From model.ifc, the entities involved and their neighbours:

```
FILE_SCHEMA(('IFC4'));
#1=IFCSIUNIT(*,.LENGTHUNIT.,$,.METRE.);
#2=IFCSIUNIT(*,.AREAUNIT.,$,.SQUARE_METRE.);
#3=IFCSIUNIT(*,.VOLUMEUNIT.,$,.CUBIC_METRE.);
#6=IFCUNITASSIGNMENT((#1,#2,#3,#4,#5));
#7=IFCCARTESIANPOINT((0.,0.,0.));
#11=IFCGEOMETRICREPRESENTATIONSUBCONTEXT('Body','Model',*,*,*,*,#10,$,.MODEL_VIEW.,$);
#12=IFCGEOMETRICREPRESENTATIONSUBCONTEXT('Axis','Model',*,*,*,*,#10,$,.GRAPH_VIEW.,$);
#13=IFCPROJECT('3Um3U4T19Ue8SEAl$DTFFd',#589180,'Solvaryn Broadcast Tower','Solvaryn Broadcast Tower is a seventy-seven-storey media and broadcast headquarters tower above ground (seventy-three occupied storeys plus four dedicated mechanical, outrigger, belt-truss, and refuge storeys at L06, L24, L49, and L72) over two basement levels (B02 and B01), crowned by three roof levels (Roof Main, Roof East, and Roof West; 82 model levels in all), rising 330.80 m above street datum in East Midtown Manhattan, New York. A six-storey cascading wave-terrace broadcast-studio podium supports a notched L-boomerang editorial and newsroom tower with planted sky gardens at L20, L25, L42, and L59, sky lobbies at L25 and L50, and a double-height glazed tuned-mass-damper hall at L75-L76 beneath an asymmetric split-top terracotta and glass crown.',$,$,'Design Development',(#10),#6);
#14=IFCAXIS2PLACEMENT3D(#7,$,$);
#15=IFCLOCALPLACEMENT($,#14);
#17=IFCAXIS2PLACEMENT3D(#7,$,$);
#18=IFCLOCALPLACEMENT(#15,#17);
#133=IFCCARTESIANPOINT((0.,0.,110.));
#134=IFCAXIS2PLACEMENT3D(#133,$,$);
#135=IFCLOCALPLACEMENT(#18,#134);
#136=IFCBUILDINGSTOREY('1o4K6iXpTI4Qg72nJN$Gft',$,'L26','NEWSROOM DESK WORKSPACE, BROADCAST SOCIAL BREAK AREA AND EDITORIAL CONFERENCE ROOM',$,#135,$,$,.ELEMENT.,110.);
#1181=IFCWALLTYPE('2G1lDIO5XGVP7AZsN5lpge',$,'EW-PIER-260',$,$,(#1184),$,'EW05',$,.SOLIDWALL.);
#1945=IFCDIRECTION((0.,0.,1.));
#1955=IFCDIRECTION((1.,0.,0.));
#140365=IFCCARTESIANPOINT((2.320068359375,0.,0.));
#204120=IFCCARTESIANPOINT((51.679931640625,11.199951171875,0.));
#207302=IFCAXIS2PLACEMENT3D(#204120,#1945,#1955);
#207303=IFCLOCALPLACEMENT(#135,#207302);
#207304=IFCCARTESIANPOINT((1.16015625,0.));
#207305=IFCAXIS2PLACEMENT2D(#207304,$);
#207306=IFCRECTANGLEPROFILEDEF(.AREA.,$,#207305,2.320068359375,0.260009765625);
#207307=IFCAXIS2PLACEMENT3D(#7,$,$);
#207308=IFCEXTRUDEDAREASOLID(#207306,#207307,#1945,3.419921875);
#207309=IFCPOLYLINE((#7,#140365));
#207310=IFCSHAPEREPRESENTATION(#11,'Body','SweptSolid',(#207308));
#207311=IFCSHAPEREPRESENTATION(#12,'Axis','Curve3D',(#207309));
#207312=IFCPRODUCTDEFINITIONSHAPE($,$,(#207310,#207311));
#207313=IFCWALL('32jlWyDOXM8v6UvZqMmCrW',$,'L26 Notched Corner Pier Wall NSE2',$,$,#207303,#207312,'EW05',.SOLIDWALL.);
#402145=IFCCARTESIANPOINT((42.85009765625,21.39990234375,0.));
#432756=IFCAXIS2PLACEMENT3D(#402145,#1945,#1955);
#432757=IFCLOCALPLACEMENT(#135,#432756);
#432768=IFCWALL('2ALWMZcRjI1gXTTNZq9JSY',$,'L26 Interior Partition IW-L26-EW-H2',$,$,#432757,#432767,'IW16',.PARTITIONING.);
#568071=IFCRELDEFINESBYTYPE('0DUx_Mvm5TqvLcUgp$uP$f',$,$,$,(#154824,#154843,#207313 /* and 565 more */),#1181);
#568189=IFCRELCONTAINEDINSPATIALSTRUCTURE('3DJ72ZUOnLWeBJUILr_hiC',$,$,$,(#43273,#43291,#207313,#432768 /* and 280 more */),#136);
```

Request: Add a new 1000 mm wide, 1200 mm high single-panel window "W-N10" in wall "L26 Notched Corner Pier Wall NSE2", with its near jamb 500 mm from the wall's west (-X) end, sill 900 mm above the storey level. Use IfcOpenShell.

```python
import numpy as np
import ifcopenshell
import ifcopenshell.api.feature
import ifcopenshell.api.geometry
import ifcopenshell.api.root
import ifcopenshell.api.spatial
import ifcopenshell.geom
import ifcopenshell.util.element
import ifcopenshell.util.placement
import ifcopenshell.util.representation
import ifcopenshell.util.shape
import ifcopenshell.util.unit

model = ifcopenshell.open("model.ifc")
unit_scale = ifcopenshell.util.unit.calculate_unit_scale(model)
settings = ifcopenshell.geom.settings()


def volume(element):
    """Net volume in cubic metres, openings subtracted."""
    shape = ifcopenshell.geom.create_shape(settings, element)
    return ifcopenshell.util.shape.get_volume(shape.geometry)


wall = model.by_guid("32jlWyDOXM8v6UvZqMmCrW")
storey = ifcopenshell.util.element.get_container(wall, ifc_class="IfcBuildingStorey")
context = ifcopenshell.util.representation.get_context(model, "Model", "Body", "MODEL_VIEW")
before = volume(wall)

width, height, from_end, sill = 1, 1.2, 0.5, 0.9  # metres

# The wall runs along its own X axis, and the end named is its -X end.
wall_shape = ifcopenshell.geom.create_shape(settings, wall)
x, y, z = ifcopenshell.util.shape.get_vertices(wall_shape.geometry).T
start = x.min() + from_end
face, thickness = float(y.min()), float(y.max() - y.min())
wall_matrix = ifcopenshell.util.placement.get_local_placement(wall.ObjectPlacement)
level = ifcopenshell.util.placement.get_local_placement(storey.ObjectPlacement)[2, 3]


def in_wall(x, y):
    """Placement at x, y metres in the wall's axes, at sill height."""
    matrix = wall_matrix.copy()
    matrix[:, 3] = wall_matrix @ np.array([x / unit_scale, y / unit_scale, 0.0, 1.0])
    matrix[2, 3] = level + sill / unit_scale
    return matrix


# Opening: a box that overshoots both wall faces by 50 mm.
opening = ifcopenshell.api.root.create_entity(model, ifc_class="IfcOpeningElement", predefined_type="OPENING")
box = ifcopenshell.api.geometry.add_wall_representation(
    model, context=context, length=width, height=height, thickness=thickness + 0.1
)
ifcopenshell.api.geometry.assign_representation(model, product=opening, representation=box)
ifcopenshell.api.geometry.edit_object_placement(model, product=opening, matrix=in_wall(start, face - 0.05), is_si=False)
ifcopenshell.api.feature.add_feature(model, feature=opening, element=wall)

window = ifcopenshell.api.root.create_entity(model, ifc_class="IfcWindow", name="W-N10", predefined_type="WINDOW")
window.OverallWidth, window.OverallHeight = width / unit_scale, height / unit_scale
window.PartitioningType = "SINGLE_PANEL"
body = ifcopenshell.api.geometry.add_window_representation(
    model,
    context=context,
    overall_width=window.OverallWidth,
    overall_height=window.OverallHeight,
    partition_type="SINGLE_PANEL",
)
ifcopenshell.api.geometry.assign_representation(model, product=window, representation=body)
ifcopenshell.api.spatial.assign_container(model, products=[window], relating_structure=storey)
ifcopenshell.api.feature.add_filling(model, opening=opening, element=window)

# Centre the window in the wall's thickness.
ifcopenshell.api.geometry.edit_object_placement(model, product=window, matrix=in_wall(start, face), is_si=False)
window_shape = ifcopenshell.geom.create_shape(settings, window)
depth = ifcopenshell.util.shape.get_vertices(window_shape.geometry)[:, 1]
offset = face + thickness / 2 - (depth.min() + depth.max()) / 2
ifcopenshell.api.geometry.edit_object_placement(model, product=window, matrix=in_wall(start, offset), is_si=False)

after = volume(wall)

print(f"wall volume {before:.3f} -> {after:.3f} m3")

model.write("model_rev.ifc")
```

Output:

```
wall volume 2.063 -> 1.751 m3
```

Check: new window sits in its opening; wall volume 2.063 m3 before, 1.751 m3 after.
